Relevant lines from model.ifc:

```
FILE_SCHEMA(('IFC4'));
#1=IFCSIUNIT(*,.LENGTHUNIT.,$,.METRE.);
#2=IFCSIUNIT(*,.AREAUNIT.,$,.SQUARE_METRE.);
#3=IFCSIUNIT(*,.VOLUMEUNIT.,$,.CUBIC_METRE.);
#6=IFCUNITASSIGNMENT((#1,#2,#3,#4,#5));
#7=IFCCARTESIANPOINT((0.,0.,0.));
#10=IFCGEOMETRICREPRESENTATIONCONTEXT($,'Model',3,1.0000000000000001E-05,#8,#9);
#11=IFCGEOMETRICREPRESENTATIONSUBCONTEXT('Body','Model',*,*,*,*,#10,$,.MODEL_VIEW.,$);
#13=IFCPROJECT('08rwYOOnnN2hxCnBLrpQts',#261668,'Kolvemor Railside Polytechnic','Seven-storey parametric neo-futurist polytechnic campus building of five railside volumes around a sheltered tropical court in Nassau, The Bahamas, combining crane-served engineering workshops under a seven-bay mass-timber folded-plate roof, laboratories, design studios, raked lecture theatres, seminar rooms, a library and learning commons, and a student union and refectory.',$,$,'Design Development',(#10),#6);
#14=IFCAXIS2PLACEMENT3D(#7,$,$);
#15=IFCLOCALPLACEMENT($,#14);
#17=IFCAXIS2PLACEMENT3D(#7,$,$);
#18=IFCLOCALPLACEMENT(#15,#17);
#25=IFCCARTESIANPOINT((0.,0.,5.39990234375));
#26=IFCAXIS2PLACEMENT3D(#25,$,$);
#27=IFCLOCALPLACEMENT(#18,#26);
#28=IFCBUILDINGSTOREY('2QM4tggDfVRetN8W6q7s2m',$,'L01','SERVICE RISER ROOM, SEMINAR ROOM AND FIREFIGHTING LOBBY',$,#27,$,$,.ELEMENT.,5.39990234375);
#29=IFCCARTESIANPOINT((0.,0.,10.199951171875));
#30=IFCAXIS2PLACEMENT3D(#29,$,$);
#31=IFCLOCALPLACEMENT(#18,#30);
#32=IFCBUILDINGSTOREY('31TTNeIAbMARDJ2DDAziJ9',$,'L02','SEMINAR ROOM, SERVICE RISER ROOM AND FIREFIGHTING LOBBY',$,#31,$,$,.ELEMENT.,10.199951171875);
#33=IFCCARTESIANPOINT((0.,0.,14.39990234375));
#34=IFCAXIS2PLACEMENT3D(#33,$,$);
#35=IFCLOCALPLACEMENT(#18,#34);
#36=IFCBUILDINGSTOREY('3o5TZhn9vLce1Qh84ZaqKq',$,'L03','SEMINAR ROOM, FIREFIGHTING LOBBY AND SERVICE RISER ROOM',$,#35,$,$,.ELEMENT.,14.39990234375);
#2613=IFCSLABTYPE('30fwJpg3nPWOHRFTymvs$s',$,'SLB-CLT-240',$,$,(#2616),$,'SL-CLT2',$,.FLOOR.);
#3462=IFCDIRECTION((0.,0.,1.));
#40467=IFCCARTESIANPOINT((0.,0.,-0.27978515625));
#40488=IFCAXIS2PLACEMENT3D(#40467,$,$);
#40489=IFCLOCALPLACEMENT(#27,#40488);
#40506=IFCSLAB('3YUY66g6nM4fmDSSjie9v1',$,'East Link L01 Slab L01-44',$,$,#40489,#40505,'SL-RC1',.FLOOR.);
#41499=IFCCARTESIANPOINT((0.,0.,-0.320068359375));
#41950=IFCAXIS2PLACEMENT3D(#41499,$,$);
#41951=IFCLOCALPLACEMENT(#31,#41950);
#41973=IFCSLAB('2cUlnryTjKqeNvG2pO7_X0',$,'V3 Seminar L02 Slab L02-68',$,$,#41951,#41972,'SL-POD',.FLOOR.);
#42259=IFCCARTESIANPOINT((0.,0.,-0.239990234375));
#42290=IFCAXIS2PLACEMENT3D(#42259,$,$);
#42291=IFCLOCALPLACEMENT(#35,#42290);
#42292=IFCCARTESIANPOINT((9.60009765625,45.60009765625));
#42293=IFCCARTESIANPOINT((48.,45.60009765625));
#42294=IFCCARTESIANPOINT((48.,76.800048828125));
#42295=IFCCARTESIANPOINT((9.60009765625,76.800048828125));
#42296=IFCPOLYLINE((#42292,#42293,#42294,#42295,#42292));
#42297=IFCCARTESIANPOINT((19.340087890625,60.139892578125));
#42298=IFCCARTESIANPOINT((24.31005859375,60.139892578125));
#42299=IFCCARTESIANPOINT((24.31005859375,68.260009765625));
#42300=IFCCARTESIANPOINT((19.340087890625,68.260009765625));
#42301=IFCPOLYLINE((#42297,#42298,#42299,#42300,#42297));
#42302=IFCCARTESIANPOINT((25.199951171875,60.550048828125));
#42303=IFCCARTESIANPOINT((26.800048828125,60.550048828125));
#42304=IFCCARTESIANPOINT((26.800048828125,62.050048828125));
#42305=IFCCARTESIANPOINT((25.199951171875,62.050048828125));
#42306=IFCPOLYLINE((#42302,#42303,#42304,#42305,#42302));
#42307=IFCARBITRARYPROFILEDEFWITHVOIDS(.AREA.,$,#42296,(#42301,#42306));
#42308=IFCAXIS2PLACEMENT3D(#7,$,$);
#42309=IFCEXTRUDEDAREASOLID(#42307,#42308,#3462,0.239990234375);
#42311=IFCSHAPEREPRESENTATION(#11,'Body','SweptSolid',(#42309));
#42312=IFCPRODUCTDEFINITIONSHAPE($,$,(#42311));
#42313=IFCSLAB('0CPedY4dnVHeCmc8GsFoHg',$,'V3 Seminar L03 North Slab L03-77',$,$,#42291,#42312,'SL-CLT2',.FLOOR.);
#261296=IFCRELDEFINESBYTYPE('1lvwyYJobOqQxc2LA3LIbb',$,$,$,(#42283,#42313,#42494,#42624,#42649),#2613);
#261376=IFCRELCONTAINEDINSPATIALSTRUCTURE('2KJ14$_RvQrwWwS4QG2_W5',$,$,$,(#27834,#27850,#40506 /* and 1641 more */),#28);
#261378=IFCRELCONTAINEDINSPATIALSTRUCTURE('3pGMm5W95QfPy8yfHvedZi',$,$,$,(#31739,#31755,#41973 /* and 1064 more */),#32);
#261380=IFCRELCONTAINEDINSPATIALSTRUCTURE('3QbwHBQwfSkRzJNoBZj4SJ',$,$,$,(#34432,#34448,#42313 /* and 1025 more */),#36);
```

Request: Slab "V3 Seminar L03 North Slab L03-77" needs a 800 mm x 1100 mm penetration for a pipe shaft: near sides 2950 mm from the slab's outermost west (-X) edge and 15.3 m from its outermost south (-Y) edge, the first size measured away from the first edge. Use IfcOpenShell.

```python
import numpy as np
import ifcopenshell
import ifcopenshell.api.feature
import ifcopenshell.api.geometry
import ifcopenshell.api.root
import ifcopenshell.geom
import ifcopenshell.util.placement
import ifcopenshell.util.representation
import ifcopenshell.util.shape
import ifcopenshell.util.unit

model = ifcopenshell.open("model.ifc")
unit_scale = ifcopenshell.util.unit.calculate_unit_scale(model)
settings = ifcopenshell.geom.settings()


def volume(element):
    """Net volume in cubic metres, openings subtracted."""
    shape = ifcopenshell.geom.create_shape(settings, element)
    return ifcopenshell.util.shape.get_volume(shape.geometry)


slab = model.by_guid("0CPedY4dnVHeCmc8GsFoHg")
before = volume(slab)

# Extent in the slab's own axes, in metres. The edges named are its -X and -Y sides.
slab_shape = ifcopenshell.geom.create_shape(settings, slab)
vertices = ifcopenshell.util.shape.get_vertices(slab_shape.geometry)
x_min, y_min, bottom = vertices.min(axis=0)
top = vertices[:, 2].max()

opening = ifcopenshell.api.root.create_entity(model, ifc_class="IfcOpeningElement", name="Pipe shaft opening", predefined_type="OPENING")
context = ifcopenshell.util.representation.get_context(model, "Model", "Body", "MODEL_VIEW")
width, depth = 0.8, 1.1
outline = [(0.0, 0.0), (width, 0.0), (width, depth), (0.0, depth), (0.0, 0.0)]
# Overshoot both faces by 50 mm so the cut is clean.
shape = ifcopenshell.api.geometry.add_slab_representation(
    model, context=context, depth=top - bottom + 0.1, polyline=outline
)
ifcopenshell.api.geometry.assign_representation(model, product=opening, representation=shape)

matrix = ifcopenshell.util.placement.get_local_placement(slab.ObjectPlacement)
matrix[:, 3] = matrix @ np.append(np.array([x_min + 2.95, y_min + 15.3, bottom - 0.05]) / unit_scale, 1.0)
ifcopenshell.api.geometry.edit_object_placement(model, product=opening, matrix=matrix, is_si=False)
ifcopenshell.api.feature.add_feature(model, feature=opening, element=slab)

after = volume(slab)

print(f"slab volume {before:.3f} -> {after:.3f} m3")

model.write("model_edited.ifc")
```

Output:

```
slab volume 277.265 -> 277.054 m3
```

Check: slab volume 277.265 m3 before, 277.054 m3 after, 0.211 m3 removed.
